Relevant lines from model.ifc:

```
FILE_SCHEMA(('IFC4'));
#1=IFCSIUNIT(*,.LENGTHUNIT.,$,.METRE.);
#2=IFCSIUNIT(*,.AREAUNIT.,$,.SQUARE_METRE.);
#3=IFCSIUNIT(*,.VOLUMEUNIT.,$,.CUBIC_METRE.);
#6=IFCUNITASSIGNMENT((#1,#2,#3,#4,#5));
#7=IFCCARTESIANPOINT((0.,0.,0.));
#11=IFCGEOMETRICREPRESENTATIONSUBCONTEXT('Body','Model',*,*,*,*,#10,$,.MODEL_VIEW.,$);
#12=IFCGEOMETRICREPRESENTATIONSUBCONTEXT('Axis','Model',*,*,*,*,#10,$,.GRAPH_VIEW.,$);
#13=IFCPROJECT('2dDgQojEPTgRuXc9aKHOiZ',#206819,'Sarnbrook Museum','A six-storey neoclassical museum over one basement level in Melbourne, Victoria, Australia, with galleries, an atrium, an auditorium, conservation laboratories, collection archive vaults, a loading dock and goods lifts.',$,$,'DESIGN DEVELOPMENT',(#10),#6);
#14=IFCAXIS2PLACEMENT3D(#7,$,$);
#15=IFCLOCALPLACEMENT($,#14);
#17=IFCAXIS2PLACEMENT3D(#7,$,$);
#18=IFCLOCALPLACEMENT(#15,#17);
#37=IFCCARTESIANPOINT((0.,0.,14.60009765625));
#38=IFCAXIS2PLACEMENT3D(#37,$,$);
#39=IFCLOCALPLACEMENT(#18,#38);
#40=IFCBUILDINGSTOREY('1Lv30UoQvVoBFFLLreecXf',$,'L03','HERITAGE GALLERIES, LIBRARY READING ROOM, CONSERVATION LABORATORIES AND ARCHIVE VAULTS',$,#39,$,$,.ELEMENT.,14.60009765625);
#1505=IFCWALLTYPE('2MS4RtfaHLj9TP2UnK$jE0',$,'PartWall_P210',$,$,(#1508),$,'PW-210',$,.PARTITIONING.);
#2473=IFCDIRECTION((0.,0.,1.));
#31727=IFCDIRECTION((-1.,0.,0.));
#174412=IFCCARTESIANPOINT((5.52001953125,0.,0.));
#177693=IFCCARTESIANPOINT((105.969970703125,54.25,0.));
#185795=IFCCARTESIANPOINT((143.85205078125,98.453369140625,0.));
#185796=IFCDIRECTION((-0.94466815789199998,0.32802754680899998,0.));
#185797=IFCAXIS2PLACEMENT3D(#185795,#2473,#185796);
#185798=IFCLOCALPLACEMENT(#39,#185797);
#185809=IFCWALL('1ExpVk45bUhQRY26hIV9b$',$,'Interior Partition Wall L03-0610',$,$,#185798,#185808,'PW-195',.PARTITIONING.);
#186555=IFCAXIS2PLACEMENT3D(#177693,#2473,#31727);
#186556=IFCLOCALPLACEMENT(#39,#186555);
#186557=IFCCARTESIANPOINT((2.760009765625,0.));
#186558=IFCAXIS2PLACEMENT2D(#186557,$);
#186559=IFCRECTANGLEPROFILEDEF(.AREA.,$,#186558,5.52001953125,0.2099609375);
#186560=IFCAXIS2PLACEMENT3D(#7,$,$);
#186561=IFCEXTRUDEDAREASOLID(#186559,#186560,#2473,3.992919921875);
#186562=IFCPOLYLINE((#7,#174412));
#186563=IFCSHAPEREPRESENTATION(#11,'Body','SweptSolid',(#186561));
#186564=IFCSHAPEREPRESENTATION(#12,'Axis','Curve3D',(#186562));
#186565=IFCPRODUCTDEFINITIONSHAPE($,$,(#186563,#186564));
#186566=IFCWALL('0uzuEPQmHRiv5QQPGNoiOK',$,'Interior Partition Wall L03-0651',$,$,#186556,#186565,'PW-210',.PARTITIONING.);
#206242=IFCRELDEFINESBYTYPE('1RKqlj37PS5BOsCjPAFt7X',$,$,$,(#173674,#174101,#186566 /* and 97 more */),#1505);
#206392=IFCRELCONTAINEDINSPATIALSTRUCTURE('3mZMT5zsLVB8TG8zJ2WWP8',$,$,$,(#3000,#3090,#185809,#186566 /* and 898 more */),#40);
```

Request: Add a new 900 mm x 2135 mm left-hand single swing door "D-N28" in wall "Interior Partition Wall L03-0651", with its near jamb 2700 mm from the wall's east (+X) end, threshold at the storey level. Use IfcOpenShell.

```python
import numpy as np
import ifcopenshell
import ifcopenshell.api.feature
import ifcopenshell.api.geometry
import ifcopenshell.api.root
import ifcopenshell.api.spatial
import ifcopenshell.geom
import ifcopenshell.util.element
import ifcopenshell.util.placement
import ifcopenshell.util.representation
import ifcopenshell.util.shape
import ifcopenshell.util.unit

model = ifcopenshell.open("model.ifc")
unit_scale = ifcopenshell.util.unit.calculate_unit_scale(model)
settings = ifcopenshell.geom.settings()


def volume(element):
    """Net volume in cubic metres, openings subtracted."""
    shape = ifcopenshell.geom.create_shape(settings, element)
    return ifcopenshell.util.shape.get_volume(shape.geometry)


wall = model.by_guid("0uzuEPQmHRiv5QQPGNoiOK")
storey = ifcopenshell.util.element.get_container(wall, ifc_class="IfcBuildingStorey")
context = ifcopenshell.util.representation.get_context(model, "Model", "Body", "MODEL_VIEW")
before = volume(wall)

width, height, from_end, sill = 0.9, 2.135, 2.7, 0.0  # metres

# The wall runs along its own X axis, and the end named is its -X end.
wall_shape = ifcopenshell.geom.create_shape(settings, wall)
x, y, z = ifcopenshell.util.shape.get_vertices(wall_shape.geometry).T
start = x.min() + from_end
face, thickness = float(y.min()), float(y.max() - y.min())
wall_matrix = ifcopenshell.util.placement.get_local_placement(wall.ObjectPlacement)
level = ifcopenshell.util.placement.get_local_placement(storey.ObjectPlacement)[2, 3]


def in_wall(x, y):
    """Placement at x, y metres in the wall's axes, at sill height."""
    matrix = wall_matrix.copy()
    matrix[:, 3] = wall_matrix @ np.array([x / unit_scale, y / unit_scale, 0.0, 1.0])
    matrix[2, 3] = level + sill / unit_scale
    return matrix


# Opening: a box that overshoots both wall faces by 50 mm.
opening = ifcopenshell.api.root.create_entity(model, ifc_class="IfcOpeningElement", predefined_type="OPENING")
box = ifcopenshell.api.geometry.add_wall_representation(
    model, context=context, length=width, height=height, thickness=thickness + 0.1
)
ifcopenshell.api.geometry.assign_representation(model, product=opening, representation=box)
ifcopenshell.api.geometry.edit_object_placement(model, product=opening, matrix=in_wall(start, face - 0.05), is_si=False)
ifcopenshell.api.feature.add_feature(model, feature=opening, element=wall)

door = ifcopenshell.api.root.create_entity(model, ifc_class="IfcDoor", name="D-N28", predefined_type="DOOR")
door.OverallWidth, door.OverallHeight = width / unit_scale, height / unit_scale
door.OperationType = "SINGLE_SWING_LEFT"
body = ifcopenshell.api.geometry.add_door_representation(
    model,
    context=context,
    overall_width=door.OverallWidth,
    overall_height=door.OverallHeight,
    operation_type="SINGLE_SWING_LEFT",
    lining_properties={"LiningDepth": thickness / unit_scale, "ThresholdDepth": thickness / unit_scale},
)
ifcopenshell.api.geometry.assign_representation(model, product=door, representation=body)
ifcopenshell.api.spatial.assign_container(model, products=[door], relating_structure=storey)
ifcopenshell.api.feature.add_filling(model, opening=opening, element=door)

# The lining spans the wall, so the door starts at the wall face.
ifcopenshell.api.geometry.edit_object_placement(model, product=door, matrix=in_wall(start, face), is_si=False)

after = volume(wall)

print(f"wall volume {before:.3f} -> {after:.3f} m3")

model.write("model_updated.ifc")
```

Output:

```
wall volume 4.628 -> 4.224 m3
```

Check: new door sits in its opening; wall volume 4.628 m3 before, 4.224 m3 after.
